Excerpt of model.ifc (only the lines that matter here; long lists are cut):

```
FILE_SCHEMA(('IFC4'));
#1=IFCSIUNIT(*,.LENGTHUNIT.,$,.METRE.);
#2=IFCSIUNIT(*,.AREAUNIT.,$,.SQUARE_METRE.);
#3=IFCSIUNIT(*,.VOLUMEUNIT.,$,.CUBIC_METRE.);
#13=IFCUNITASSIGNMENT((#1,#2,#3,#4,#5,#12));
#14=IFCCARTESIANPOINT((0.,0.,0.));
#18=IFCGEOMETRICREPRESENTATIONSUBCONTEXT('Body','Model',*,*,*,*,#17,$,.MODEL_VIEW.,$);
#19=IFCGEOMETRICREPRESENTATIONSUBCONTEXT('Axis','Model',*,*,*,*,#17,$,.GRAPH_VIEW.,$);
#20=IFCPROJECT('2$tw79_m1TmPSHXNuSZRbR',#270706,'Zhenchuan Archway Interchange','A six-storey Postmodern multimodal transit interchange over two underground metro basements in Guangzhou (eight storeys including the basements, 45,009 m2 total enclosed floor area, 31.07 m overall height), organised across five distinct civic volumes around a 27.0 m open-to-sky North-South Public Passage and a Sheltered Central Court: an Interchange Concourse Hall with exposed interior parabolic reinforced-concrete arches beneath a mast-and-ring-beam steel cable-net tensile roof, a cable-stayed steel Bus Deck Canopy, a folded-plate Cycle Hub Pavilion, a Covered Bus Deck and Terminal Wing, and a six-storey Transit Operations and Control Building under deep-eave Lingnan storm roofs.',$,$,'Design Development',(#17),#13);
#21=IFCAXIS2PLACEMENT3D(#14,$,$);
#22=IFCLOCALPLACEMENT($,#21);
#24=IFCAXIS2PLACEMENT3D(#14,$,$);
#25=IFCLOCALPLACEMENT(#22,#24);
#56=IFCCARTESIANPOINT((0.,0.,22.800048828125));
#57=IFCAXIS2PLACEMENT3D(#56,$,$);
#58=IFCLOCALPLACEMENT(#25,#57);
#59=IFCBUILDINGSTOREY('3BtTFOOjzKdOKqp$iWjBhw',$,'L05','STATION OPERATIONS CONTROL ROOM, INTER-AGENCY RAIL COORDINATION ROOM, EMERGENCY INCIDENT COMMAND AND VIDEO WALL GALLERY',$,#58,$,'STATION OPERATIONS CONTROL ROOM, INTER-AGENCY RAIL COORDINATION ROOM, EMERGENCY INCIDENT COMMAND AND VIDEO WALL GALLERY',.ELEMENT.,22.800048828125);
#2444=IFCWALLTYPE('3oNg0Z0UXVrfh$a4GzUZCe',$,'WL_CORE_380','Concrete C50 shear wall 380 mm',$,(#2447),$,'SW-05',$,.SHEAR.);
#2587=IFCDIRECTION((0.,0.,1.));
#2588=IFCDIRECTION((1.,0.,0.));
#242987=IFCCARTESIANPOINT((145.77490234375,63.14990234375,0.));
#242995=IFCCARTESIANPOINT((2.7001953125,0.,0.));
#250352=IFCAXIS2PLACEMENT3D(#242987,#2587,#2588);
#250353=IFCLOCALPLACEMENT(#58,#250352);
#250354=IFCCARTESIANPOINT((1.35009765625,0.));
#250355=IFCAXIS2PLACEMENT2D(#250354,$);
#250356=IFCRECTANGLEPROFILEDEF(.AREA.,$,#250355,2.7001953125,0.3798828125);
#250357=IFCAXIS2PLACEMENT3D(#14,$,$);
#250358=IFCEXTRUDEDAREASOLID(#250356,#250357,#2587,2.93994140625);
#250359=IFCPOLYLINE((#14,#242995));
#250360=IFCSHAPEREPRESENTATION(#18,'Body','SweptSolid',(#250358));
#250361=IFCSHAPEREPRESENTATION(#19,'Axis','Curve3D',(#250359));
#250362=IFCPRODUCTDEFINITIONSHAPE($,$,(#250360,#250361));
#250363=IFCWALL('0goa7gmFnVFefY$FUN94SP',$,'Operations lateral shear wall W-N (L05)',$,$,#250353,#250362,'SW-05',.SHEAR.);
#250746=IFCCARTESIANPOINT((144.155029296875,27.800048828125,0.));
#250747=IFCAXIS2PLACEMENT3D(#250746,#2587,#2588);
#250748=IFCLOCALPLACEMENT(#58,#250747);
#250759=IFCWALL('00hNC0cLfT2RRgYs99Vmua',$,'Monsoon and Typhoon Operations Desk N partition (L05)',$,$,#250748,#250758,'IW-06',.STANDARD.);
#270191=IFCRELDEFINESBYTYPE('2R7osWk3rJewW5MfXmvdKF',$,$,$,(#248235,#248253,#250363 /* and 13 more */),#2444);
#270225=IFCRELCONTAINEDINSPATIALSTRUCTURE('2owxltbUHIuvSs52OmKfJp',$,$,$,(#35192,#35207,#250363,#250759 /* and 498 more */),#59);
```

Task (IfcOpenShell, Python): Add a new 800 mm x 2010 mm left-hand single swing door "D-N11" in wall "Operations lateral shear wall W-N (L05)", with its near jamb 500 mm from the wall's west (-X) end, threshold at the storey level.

```python
import numpy as np
import ifcopenshell
import ifcopenshell.api.feature
import ifcopenshell.api.geometry
import ifcopenshell.api.root
import ifcopenshell.api.spatial
import ifcopenshell.geom
import ifcopenshell.util.element
import ifcopenshell.util.placement
import ifcopenshell.util.representation
import ifcopenshell.util.shape
import ifcopenshell.util.unit

model = ifcopenshell.open("model.ifc")
unit_scale = ifcopenshell.util.unit.calculate_unit_scale(model)
settings = ifcopenshell.geom.settings()


def volume(element):
    """Net volume in cubic metres, openings subtracted."""
    shape = ifcopenshell.geom.create_shape(settings, element)
    return ifcopenshell.util.shape.get_volume(shape.geometry)


wall = model.by_id(250363)
storey = ifcopenshell.util.element.get_container(wall, ifc_class="IfcBuildingStorey")
context = ifcopenshell.util.representation.get_context(model, "Model", "Body", "MODEL_VIEW")
before = volume(wall)

width, height, from_end, sill = 0.8, 2.01, 0.5, 0.0  # metres

# The wall runs along its own X axis, and the end named is its -X end.
wall_shape = ifcopenshell.geom.create_shape(settings, wall)
x, y, z = ifcopenshell.util.shape.get_vertices(wall_shape.geometry).T
start = x.min() + from_end
face, thickness = float(y.min()), float(y.max() - y.min())
wall_matrix = ifcopenshell.util.placement.get_local_placement(wall.ObjectPlacement)
level = ifcopenshell.util.placement.get_local_placement(storey.ObjectPlacement)[2, 3]


def in_wall(x, y):
    """Placement at x, y metres in the wall's axes, at sill height."""
    matrix = wall_matrix.copy()
    matrix[:, 3] = wall_matrix @ np.array([x / unit_scale, y / unit_scale, 0.0, 1.0])
    matrix[2, 3] = level + sill / unit_scale
    return matrix


# Opening: a box that overshoots both wall faces by 50 mm.
opening = ifcopenshell.api.root.create_entity(model, ifc_class="IfcOpeningElement", predefined_type="OPENING")
box = ifcopenshell.api.geometry.add_wall_representation(
    model, context=context, length=width, height=height, thickness=thickness + 0.1
)
ifcopenshell.api.geometry.assign_representation(model, product=opening, representation=box)
ifcopenshell.api.geometry.edit_object_placement(model, product=opening, matrix=in_wall(start, face - 0.05), is_si=False)
ifcopenshell.api.feature.add_feature(model, feature=opening, element=wall)

door = ifcopenshell.api.root.create_entity(model, ifc_class="IfcDoor", name="D-N11", predefined_type="DOOR")
door.OverallWidth, door.OverallHeight = width / unit_scale, height / unit_scale
door.OperationType = "SINGLE_SWING_LEFT"
body = ifcopenshell.api.geometry.add_door_representation(
    model,
    context=context,
    overall_width=door.OverallWidth,
    overall_height=door.OverallHeight,
    operation_type="SINGLE_SWING_LEFT",
    lining_properties={"LiningDepth": thickness / unit_scale, "ThresholdDepth": thickness / unit_scale},
)
ifcopenshell.api.geometry.assign_representation(model, product=door, representation=body)
ifcopenshell.api.spatial.assign_container(model, products=[door], relating_structure=storey)
ifcopenshell.api.feature.add_filling(model, opening=opening, element=door)

# The lining spans the wall, so the door starts at the wall face.
ifcopenshell.api.geometry.edit_object_placement(model, product=door, matrix=in_wall(start, face), is_si=False)

after = volume(wall)

print(f"wall volume {before:.3f} -> {after:.3f} m3")

model.write("model_v2.ifc")
```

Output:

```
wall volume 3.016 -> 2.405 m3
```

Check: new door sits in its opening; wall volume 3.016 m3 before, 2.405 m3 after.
